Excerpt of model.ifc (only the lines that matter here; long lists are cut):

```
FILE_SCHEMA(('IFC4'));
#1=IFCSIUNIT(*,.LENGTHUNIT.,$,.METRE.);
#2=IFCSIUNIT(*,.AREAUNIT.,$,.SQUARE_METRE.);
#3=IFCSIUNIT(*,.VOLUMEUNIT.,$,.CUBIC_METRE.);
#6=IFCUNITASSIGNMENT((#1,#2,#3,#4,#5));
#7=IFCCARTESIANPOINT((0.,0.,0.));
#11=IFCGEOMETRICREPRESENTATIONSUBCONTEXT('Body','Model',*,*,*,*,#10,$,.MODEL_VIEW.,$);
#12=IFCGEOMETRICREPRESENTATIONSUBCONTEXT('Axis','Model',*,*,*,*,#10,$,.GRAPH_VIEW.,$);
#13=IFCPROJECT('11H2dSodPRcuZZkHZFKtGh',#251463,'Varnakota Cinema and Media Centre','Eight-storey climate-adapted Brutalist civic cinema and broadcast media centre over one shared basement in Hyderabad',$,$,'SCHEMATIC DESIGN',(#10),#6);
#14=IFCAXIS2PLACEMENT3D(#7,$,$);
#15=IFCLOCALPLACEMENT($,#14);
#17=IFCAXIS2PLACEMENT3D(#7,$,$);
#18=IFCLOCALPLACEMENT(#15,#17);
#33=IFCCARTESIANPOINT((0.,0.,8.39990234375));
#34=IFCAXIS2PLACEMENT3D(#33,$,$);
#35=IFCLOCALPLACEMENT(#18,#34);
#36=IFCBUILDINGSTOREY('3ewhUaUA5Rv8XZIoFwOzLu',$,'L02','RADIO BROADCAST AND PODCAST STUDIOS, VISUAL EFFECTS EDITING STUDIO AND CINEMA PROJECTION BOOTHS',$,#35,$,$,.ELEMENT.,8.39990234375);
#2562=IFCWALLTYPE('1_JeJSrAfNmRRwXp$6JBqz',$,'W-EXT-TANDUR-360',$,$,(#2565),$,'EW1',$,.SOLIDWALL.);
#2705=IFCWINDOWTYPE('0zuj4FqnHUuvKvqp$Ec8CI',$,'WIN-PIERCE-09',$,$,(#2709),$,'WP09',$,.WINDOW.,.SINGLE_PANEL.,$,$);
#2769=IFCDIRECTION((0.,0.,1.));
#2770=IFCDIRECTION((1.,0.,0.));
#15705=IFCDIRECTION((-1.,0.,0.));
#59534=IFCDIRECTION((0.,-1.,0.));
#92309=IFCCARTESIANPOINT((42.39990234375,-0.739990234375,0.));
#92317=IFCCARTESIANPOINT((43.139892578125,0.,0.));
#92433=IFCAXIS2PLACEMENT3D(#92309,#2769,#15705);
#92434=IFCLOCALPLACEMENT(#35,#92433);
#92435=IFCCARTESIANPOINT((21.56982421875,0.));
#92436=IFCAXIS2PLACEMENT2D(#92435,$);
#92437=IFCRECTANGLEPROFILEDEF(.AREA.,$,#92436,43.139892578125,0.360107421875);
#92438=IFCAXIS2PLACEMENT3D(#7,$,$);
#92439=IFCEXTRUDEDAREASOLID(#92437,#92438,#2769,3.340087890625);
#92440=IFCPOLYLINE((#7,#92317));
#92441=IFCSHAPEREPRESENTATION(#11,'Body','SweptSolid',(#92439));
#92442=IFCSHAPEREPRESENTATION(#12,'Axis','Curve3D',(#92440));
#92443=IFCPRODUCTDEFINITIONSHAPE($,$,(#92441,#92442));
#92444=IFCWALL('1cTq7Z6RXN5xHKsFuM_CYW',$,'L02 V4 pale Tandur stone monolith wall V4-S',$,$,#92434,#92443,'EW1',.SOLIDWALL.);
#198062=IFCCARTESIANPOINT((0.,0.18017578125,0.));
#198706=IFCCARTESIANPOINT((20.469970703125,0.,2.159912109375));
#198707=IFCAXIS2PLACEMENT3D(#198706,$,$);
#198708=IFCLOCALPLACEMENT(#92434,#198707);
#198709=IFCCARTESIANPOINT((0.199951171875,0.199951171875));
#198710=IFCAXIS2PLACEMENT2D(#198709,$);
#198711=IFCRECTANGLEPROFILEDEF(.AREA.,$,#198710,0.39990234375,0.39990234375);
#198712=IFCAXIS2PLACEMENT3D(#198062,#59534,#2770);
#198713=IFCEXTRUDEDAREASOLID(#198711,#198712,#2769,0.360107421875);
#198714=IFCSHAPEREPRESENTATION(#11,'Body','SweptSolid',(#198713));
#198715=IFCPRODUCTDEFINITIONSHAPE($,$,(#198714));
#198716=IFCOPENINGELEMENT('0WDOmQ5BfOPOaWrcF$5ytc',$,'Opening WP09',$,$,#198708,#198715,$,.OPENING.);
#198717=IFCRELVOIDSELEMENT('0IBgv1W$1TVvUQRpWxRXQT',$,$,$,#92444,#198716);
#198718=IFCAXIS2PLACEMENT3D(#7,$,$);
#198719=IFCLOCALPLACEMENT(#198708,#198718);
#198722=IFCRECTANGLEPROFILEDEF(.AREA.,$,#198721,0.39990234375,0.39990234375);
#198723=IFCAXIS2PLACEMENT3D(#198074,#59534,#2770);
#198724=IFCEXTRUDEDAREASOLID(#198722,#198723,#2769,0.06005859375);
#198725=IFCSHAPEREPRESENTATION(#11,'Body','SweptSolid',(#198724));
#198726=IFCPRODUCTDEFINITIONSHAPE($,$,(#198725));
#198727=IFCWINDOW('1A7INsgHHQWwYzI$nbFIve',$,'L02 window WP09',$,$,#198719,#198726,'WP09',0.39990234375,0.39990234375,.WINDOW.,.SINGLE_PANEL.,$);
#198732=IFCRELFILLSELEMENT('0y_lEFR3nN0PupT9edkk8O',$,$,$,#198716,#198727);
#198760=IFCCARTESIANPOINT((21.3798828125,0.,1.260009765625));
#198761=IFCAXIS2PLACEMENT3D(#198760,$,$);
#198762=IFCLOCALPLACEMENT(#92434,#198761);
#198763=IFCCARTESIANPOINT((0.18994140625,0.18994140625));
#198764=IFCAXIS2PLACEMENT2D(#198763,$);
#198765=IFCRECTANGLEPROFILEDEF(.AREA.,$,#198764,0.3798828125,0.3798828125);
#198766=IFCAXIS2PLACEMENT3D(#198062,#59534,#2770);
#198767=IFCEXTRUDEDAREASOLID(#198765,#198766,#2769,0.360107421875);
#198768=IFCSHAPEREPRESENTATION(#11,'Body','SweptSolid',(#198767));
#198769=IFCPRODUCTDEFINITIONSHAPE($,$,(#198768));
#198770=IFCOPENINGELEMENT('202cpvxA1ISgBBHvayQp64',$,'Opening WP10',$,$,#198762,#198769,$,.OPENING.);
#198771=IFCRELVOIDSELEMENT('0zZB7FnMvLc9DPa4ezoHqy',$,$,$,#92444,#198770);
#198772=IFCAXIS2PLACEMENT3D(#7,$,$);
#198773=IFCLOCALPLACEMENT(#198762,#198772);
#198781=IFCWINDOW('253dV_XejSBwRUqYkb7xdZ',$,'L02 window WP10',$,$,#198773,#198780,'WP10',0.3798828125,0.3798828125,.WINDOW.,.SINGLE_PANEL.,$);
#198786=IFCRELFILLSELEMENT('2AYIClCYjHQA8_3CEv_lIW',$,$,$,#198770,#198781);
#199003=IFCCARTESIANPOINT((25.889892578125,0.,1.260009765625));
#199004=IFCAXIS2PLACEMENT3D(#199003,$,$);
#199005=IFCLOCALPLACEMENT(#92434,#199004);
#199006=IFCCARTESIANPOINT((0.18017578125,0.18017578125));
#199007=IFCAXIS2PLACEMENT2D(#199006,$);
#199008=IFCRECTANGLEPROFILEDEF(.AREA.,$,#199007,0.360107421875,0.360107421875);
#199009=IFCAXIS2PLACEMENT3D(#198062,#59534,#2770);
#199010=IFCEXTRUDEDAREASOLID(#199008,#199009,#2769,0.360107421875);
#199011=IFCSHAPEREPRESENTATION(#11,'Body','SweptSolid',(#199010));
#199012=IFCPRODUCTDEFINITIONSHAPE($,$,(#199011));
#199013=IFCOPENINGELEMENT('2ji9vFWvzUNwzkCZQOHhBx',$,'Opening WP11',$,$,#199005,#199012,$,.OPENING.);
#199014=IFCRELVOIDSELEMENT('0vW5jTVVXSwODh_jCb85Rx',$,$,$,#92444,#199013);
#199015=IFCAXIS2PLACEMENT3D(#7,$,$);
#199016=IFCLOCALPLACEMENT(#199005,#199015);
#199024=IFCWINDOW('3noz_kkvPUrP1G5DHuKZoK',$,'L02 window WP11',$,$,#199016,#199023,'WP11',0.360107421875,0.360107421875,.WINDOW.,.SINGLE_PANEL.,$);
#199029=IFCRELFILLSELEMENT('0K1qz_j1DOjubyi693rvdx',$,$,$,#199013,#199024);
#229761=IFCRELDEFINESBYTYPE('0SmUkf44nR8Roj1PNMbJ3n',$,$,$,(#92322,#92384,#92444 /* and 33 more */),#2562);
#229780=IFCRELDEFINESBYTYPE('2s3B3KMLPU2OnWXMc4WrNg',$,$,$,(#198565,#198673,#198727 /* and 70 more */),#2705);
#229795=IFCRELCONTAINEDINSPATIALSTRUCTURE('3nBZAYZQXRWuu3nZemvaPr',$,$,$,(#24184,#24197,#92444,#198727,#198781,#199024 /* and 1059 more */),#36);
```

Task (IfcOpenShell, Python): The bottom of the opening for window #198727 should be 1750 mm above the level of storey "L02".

```python
import numpy as np
import ifcopenshell
import ifcopenshell.api.geometry
import ifcopenshell.geom
import ifcopenshell.util.element
import ifcopenshell.util.placement
import ifcopenshell.util.shape
import ifcopenshell.util.unit

model = ifcopenshell.open("model.ifc")
unit_scale = ifcopenshell.util.unit.calculate_unit_scale(model)

window = model.by_id(198727)
opening = window.FillsVoids[0].RelatingOpeningElement
storey = ifcopenshell.util.element.get_container(window, ifc_class="IfcBuildingStorey")
level = ifcopenshell.util.placement.get_local_placement(storey.ObjectPlacement)[2, 3]

# The opening's origin need not be at the sill, so measure its lowest point.
shape = ifcopenshell.geom.create_shape(ifcopenshell.geom.settings(), opening)
bottom = ifcopenshell.util.shape.get_shape_bottom_elevation(shape, shape.geometry) / unit_scale
dz = level + 1.75 / unit_scale - bottom

shift = np.array([0.0, 0.0, dz])
# The window is placed relative to its opening, so it follows when the opening moves.
matrix = ifcopenshell.util.placement.get_local_placement(opening.ObjectPlacement)
matrix[:3, 3] += shift
ifcopenshell.api.geometry.edit_object_placement(
    model, product=opening, matrix=matrix, is_si=False, should_transform_children=True
)

print(f"moved by {dz * unit_scale:+.3f} m")

model.write("model_edited.ifc")
```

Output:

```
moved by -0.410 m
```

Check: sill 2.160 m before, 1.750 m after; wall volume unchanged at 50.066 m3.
